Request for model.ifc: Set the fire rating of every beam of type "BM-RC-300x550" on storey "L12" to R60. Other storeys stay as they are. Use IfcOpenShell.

First a look at what the model holds.

```python
import ifcopenshell
import ifcopenshell.util.element

model = ifcopenshell.open("model.ifc")
print(model.schema)
storey = next(s for s in model.by_type("IfcBuildingStorey") if s.Name == "L12")
beams = [e for e in ifcopenshell.util.element.get_decomposition(storey) if e.is_a("IfcBeam")]
seen = {}
for e in beams:
    element_type = ifcopenshell.util.element.get_type(e)
    key = (element_type.Name if element_type != e and element_type else None, ifcopenshell.util.element.get_pset(e, "Pset_BeamCommon", "FireRating"))
    seen[key] = seen.get(key, 0) + 1
for (name, value), count in sorted(seen.items(), key=str):
    print(count, "x", name, "|", value)
```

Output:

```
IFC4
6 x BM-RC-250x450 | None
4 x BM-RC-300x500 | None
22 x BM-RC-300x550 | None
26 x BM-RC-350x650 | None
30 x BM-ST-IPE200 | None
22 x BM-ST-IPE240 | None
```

```python
import ifcopenshell
import ifcopenshell.api.pset
import ifcopenshell.util.element

model = ifcopenshell.open("model.ifc")

storey = next(s for s in model.by_type("IfcBuildingStorey") if s.Name == "L12")
beams = [e for e in ifcopenshell.util.element.get_decomposition(storey) if e.is_a("IfcBeam")]

count = 0
for e in beams:
    element_type = ifcopenshell.util.element.get_type(e)
    if element_type in (None, e) or element_type.Name != "BM-RC-300x550":
        continue
    # add_pset returns the element's existing set when there is one.
    pset = ifcopenshell.api.pset.add_pset(model, product=e, name="Pset_BeamCommon")
    ifcopenshell.api.pset.edit_pset(model, pset=pset, properties={"FireRating": "R60"})
    count += 1

print(count, "beams updated")

model.write("model_v2.ifc")
```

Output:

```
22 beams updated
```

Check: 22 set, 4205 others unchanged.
